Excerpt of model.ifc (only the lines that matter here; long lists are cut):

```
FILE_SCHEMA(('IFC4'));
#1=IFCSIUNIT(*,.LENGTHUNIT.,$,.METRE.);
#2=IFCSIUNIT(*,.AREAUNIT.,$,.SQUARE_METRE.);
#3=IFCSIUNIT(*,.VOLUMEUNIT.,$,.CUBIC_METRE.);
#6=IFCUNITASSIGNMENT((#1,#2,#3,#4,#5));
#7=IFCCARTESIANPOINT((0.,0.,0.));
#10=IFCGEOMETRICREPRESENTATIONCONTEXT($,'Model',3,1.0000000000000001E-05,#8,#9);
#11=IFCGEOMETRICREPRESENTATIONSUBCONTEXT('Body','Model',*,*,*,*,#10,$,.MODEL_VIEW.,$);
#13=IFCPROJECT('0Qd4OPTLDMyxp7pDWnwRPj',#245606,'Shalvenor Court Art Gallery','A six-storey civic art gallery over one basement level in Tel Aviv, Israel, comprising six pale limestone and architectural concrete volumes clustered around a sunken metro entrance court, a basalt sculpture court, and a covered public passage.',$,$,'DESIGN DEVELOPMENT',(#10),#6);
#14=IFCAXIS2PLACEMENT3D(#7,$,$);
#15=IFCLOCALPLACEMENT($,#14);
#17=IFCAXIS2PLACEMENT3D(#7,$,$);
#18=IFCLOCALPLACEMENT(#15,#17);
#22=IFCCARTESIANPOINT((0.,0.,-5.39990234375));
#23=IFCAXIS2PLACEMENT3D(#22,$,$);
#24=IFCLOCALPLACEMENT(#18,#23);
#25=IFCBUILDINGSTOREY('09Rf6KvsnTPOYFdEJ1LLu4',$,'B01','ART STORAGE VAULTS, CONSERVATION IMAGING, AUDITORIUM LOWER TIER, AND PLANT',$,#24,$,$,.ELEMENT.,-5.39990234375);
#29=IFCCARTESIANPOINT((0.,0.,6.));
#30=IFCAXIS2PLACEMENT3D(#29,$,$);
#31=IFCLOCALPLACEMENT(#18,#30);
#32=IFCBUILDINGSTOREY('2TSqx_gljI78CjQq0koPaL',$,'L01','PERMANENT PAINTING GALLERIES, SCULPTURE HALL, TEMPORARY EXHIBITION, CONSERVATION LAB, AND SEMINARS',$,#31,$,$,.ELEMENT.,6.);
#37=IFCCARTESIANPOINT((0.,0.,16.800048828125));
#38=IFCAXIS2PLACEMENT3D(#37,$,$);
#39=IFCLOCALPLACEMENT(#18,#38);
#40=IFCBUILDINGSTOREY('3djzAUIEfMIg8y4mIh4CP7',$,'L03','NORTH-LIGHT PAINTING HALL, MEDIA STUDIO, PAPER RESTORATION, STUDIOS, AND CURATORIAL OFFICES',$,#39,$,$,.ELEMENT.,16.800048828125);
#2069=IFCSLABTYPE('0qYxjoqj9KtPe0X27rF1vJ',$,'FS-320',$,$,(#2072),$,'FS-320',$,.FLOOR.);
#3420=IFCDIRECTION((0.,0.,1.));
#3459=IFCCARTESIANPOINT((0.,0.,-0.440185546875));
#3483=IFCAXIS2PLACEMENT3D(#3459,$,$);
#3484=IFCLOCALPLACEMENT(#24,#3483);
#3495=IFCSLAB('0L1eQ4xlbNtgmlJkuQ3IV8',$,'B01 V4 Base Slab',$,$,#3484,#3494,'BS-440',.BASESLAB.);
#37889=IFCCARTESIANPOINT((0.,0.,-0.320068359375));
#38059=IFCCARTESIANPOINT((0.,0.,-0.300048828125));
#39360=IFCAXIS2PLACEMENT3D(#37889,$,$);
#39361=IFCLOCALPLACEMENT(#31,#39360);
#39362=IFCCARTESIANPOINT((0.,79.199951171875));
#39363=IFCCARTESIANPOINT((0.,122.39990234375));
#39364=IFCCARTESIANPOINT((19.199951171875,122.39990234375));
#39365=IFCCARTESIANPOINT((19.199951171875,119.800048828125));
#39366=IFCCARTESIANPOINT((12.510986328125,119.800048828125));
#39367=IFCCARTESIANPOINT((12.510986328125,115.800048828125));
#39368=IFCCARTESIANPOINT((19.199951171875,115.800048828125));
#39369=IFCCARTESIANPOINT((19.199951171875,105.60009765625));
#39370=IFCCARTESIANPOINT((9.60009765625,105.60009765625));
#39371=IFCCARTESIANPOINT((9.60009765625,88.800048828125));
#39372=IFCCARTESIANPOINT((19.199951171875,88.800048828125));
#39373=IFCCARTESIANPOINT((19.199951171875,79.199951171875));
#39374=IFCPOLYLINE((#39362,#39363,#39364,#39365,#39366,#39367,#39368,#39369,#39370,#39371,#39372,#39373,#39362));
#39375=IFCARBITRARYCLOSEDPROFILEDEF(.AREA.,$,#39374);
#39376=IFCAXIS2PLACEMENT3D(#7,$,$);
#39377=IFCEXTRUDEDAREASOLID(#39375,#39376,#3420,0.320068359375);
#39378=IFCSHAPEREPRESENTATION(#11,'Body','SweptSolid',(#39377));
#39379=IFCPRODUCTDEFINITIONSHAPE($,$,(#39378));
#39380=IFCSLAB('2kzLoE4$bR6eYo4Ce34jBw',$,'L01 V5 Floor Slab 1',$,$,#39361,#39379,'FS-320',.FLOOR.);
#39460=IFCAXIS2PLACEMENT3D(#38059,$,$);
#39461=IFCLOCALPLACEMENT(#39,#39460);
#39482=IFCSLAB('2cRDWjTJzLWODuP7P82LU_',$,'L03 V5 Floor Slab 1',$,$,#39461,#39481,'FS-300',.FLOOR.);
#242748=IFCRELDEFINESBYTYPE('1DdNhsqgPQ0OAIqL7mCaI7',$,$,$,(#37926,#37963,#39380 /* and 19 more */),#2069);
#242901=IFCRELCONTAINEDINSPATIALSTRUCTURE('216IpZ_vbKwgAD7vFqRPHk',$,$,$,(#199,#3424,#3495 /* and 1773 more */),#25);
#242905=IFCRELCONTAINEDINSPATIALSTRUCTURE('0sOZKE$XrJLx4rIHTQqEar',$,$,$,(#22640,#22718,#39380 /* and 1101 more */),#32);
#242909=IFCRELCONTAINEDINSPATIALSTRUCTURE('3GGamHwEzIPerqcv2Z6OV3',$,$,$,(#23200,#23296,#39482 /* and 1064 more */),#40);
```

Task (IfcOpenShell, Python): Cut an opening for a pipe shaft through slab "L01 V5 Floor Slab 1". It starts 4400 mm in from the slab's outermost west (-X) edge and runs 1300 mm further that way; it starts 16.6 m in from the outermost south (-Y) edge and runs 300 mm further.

```python
import numpy as np
import ifcopenshell
import ifcopenshell.api.feature
import ifcopenshell.api.geometry
import ifcopenshell.api.root
import ifcopenshell.geom
import ifcopenshell.util.placement
import ifcopenshell.util.representation
import ifcopenshell.util.shape
import ifcopenshell.util.unit

model = ifcopenshell.open("model.ifc")
unit_scale = ifcopenshell.util.unit.calculate_unit_scale(model)
settings = ifcopenshell.geom.settings()


def volume(element):
    """Net volume in cubic metres, openings subtracted."""
    shape = ifcopenshell.geom.create_shape(settings, element)
    return ifcopenshell.util.shape.get_volume(shape.geometry)


slab = model.by_id(39380)
before = volume(slab)

# Extent in the slab's own axes, in metres. The edges named are its -X and -Y sides.
slab_shape = ifcopenshell.geom.create_shape(settings, slab)
vertices = ifcopenshell.util.shape.get_vertices(slab_shape.geometry)
x_min, y_min, bottom = vertices.min(axis=0)
top = vertices[:, 2].max()

opening = ifcopenshell.api.root.create_entity(model, ifc_class="IfcOpeningElement", name="Pipe shaft opening", predefined_type="OPENING")
context = ifcopenshell.util.representation.get_context(model, "Model", "Body", "MODEL_VIEW")
width, depth = 1.3, 0.3
outline = [(0.0, 0.0), (width, 0.0), (width, depth), (0.0, depth), (0.0, 0.0)]
# Overshoot both faces by 50 mm so the cut is clean.
shape = ifcopenshell.api.geometry.add_slab_representation(
    model, context=context, depth=top - bottom + 0.1, polyline=outline
)
ifcopenshell.api.geometry.assign_representation(model, product=opening, representation=shape)

matrix = ifcopenshell.util.placement.get_local_placement(slab.ObjectPlacement)
matrix[:, 3] = matrix @ np.append(np.array([x_min + 4.4, y_min + 16.6, bottom - 0.05]) / unit_scale, 1.0)
ifcopenshell.api.geometry.edit_object_placement(model, product=opening, matrix=matrix, is_si=False)
ifcopenshell.api.feature.add_feature(model, feature=opening, element=slab)

after = volume(slab)

print(f"slab volume {before:.3f} -> {after:.3f} m3")

model.write("model_updated.ifc")
```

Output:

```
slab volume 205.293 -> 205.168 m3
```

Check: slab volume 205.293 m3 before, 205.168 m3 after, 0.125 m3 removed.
